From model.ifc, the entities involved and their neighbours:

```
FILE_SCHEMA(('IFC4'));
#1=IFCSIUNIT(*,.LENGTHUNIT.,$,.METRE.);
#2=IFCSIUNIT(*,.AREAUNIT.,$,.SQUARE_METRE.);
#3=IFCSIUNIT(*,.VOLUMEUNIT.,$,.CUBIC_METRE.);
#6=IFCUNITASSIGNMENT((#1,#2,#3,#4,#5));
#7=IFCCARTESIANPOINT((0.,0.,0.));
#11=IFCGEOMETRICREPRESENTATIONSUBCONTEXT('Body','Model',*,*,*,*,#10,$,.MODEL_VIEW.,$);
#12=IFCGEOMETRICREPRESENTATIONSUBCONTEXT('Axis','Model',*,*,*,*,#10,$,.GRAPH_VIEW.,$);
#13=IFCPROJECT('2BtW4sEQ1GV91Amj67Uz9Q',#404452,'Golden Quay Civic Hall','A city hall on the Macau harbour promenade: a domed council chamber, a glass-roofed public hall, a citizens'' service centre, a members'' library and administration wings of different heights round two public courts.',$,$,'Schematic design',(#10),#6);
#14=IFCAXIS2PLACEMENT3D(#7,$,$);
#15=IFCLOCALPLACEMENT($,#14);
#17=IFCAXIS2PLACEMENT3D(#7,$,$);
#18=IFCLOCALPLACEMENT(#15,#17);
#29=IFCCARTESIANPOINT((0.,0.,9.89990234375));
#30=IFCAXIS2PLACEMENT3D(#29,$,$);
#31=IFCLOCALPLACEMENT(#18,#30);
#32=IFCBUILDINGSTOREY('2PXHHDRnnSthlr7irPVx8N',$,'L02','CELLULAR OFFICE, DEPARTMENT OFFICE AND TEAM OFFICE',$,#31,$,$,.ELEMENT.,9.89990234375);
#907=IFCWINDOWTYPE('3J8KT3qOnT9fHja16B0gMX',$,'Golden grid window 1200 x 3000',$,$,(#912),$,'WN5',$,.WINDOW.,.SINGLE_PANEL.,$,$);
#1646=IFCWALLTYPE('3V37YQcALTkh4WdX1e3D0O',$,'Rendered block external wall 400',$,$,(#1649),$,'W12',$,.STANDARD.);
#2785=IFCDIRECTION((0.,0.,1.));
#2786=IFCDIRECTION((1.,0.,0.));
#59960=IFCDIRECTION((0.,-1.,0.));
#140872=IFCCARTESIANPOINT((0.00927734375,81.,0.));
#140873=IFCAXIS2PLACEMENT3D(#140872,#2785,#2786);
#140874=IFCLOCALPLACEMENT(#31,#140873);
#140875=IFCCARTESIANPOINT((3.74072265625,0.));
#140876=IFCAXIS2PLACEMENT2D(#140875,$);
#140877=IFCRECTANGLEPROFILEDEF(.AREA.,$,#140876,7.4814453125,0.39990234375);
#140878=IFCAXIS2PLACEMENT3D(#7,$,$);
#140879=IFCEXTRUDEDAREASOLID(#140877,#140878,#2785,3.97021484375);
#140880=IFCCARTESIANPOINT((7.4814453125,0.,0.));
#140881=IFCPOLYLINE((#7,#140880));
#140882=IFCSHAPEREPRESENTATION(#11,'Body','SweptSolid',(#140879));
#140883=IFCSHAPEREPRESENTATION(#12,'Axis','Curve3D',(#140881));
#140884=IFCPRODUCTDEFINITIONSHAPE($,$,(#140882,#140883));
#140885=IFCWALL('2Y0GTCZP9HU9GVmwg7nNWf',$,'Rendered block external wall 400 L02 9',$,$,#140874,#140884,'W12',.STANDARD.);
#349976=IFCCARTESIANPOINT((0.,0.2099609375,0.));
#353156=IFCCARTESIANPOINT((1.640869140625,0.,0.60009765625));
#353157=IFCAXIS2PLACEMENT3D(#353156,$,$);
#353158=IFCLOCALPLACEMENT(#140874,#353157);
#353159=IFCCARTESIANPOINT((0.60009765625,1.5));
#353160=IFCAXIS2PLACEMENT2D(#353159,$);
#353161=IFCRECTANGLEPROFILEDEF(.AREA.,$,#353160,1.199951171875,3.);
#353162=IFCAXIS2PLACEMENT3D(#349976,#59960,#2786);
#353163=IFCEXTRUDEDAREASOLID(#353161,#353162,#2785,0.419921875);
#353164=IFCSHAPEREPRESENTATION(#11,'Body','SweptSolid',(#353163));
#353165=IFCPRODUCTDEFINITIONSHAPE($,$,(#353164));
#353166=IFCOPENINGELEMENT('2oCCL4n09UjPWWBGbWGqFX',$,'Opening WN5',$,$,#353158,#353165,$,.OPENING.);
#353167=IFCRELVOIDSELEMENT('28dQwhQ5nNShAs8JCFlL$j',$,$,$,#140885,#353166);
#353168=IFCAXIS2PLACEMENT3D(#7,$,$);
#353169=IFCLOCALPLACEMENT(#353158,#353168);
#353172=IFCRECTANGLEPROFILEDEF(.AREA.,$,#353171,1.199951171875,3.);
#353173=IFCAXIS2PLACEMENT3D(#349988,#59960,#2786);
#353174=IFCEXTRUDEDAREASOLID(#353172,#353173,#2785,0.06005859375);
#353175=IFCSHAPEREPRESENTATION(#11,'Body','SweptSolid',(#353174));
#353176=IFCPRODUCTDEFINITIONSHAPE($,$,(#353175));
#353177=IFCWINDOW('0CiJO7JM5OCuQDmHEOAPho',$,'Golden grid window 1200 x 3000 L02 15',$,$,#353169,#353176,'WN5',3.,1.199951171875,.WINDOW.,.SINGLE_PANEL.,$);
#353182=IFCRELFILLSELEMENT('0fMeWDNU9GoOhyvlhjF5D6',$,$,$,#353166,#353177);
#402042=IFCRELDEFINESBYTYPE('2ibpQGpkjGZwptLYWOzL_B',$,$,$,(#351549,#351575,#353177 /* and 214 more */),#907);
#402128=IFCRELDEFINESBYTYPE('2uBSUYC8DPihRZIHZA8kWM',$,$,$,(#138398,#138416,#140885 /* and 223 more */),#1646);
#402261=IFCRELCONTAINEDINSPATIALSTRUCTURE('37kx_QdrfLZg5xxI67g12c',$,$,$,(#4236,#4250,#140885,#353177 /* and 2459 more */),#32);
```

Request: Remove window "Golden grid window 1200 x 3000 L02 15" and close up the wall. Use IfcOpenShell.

```python
import ifcopenshell
import ifcopenshell.api.feature
import ifcopenshell.api.root
import ifcopenshell.geom
import ifcopenshell.util.shape

model = ifcopenshell.open("model.ifc")
settings = ifcopenshell.geom.settings()


def volume(element):
    """Net volume in cubic metres, openings subtracted."""
    shape = ifcopenshell.geom.create_shape(settings, element)
    return ifcopenshell.util.shape.get_volume(shape.geometry)


window = model.by_guid("0CiJO7JM5OCuQDmHEOAPho")
opening = window.FillsVoids[0].RelatingOpeningElement
wall = opening.VoidsElements[0].RelatingBuildingElement
before = volume(wall)

ifcopenshell.api.root.remove_product(model, product=window)
ifcopenshell.api.feature.remove_feature(model, feature=opening)

after = volume(wall)

print(f"wall volume {before:.3f} -> {after:.3f} m3")

model.write("model_edited.ifc")
```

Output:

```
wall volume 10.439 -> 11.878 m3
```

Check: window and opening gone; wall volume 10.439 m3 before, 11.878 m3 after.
